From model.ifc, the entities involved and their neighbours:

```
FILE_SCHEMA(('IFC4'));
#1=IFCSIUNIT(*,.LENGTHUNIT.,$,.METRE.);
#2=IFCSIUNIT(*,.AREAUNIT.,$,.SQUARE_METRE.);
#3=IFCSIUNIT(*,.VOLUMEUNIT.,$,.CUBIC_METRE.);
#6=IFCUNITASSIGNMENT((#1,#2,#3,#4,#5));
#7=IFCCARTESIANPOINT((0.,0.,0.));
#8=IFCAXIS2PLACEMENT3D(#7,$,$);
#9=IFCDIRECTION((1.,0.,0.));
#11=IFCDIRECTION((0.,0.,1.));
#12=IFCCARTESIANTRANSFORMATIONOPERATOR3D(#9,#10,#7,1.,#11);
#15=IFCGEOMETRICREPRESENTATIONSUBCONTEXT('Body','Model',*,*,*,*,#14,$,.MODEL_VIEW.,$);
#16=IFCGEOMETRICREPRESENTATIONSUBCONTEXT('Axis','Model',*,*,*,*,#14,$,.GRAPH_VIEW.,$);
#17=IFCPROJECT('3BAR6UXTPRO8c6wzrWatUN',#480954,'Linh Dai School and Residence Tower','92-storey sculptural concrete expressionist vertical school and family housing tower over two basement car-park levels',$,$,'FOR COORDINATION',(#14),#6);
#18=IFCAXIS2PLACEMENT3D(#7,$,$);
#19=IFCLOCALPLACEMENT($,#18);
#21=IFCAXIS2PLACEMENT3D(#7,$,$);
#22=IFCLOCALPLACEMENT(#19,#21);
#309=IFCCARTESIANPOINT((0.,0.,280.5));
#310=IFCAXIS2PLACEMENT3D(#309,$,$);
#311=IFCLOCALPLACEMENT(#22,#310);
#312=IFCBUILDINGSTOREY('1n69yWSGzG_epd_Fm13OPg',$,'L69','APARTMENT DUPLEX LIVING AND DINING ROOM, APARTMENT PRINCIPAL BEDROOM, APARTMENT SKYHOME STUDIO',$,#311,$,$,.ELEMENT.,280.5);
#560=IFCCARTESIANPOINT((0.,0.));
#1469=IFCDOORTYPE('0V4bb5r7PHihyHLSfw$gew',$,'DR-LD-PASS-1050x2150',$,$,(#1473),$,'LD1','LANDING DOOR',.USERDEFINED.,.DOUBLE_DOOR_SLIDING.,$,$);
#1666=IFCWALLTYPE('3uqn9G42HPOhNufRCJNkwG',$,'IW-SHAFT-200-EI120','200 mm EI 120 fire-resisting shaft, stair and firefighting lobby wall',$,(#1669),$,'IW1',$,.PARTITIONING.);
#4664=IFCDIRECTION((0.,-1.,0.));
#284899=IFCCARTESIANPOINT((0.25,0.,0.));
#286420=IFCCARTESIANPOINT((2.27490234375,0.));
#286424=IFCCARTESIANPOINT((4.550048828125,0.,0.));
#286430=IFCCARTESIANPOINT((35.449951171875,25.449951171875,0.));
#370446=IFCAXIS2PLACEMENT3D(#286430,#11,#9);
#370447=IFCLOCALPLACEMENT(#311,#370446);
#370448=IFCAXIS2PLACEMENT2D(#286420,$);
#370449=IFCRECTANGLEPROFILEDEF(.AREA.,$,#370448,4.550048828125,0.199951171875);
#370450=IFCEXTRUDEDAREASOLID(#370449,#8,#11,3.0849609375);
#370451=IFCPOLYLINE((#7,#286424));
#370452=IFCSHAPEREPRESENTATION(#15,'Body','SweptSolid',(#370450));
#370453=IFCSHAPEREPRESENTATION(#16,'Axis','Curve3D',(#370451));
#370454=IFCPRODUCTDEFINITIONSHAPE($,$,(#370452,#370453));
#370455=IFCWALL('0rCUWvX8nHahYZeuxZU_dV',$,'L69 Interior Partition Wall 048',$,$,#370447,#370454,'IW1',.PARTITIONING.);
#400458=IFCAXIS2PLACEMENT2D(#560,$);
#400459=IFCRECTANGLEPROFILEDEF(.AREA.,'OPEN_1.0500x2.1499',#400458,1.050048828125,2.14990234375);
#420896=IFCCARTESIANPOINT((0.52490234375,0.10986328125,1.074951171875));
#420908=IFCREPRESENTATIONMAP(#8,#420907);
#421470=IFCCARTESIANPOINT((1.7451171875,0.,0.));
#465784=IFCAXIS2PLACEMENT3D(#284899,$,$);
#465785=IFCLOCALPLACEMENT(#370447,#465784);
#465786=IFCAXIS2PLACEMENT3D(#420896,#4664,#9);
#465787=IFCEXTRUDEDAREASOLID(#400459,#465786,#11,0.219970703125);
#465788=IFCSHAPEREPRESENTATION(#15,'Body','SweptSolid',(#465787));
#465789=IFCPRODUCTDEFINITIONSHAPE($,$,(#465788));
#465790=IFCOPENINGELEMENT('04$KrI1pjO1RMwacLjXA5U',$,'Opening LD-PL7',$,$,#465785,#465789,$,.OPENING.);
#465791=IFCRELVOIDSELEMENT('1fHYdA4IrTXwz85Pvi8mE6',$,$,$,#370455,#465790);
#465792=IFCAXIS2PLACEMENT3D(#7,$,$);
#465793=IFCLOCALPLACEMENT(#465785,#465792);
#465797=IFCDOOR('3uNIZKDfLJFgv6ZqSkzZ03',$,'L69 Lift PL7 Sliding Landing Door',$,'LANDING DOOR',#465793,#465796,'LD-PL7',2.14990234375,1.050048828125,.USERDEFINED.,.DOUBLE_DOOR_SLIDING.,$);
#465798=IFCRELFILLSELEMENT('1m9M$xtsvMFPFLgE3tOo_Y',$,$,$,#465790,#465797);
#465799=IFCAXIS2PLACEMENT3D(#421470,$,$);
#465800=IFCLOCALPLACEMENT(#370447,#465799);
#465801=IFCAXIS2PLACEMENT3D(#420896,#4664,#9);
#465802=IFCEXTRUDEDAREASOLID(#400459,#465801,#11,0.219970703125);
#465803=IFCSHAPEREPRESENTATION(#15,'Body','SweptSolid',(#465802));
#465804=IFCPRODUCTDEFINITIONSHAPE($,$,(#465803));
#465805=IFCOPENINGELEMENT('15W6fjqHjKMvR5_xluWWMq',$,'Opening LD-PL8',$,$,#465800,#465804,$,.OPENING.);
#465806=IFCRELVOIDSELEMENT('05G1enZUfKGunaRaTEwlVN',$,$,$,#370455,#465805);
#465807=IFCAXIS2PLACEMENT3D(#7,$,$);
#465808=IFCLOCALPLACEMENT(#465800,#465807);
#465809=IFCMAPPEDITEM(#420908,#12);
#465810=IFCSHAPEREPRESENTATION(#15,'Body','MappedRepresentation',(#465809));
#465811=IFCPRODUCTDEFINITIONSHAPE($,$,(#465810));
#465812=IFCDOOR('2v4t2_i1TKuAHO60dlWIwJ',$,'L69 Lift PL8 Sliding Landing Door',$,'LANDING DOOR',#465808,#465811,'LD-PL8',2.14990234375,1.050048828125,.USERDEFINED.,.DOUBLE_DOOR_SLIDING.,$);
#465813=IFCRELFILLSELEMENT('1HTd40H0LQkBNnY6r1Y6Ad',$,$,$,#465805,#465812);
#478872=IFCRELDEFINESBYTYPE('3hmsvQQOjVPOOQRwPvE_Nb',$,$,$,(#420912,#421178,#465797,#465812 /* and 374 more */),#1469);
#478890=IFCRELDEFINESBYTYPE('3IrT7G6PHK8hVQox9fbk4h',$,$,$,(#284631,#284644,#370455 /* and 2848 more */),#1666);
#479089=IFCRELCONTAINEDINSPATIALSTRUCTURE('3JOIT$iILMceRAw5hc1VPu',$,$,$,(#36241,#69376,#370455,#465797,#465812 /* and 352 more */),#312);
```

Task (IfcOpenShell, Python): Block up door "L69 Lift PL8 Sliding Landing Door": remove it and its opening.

```python
import ifcopenshell
import ifcopenshell.api.feature
import ifcopenshell.api.root
import ifcopenshell.geom
import ifcopenshell.util.shape

model = ifcopenshell.open("model.ifc")
settings = ifcopenshell.geom.settings()


def volume(element):
    """Net volume in cubic metres, openings subtracted."""
    shape = ifcopenshell.geom.create_shape(settings, element)
    return ifcopenshell.util.shape.get_volume(shape.geometry)


door = model.by_guid("2v4t2_i1TKuAHO60dlWIwJ")
opening = door.FillsVoids[0].RelatingOpeningElement
wall = opening.VoidsElements[0].RelatingBuildingElement
before = volume(wall)

ifcopenshell.api.root.remove_product(model, product=door)
ifcopenshell.api.feature.remove_feature(model, feature=opening)

after = volume(wall)

print(f"wall volume {before:.3f} -> {after:.3f} m3")

model.write("model_rev.ifc")
```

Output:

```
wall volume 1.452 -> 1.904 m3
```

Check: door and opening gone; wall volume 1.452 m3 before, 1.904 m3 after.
